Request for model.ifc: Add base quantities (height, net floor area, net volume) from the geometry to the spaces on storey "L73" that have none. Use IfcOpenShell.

First a look at what the model holds.

```python
import ifcopenshell
import ifcopenshell.util.element
import ifcopenshell.util.unit

model = ifcopenshell.open("model.ifc")
print(model.schema)
for unit_type in ("LENGTHUNIT", "AREAUNIT", "VOLUMEUNIT"):
    print(unit_type, ifcopenshell.util.unit.calculate_unit_scale(model, unit_type))
storey = next(s for s in model.by_type("IfcBuildingStorey") if s.Name == "L73")
spaces = [e for e in ifcopenshell.util.element.get_decomposition(storey) if e.is_a("IfcSpace")]
for e in sorted(spaces, key=lambda e: e.id()):
    print(e.id(), e.is_a(), e.Name, list(ifcopenshell.util.element.get_psets(e, qtos_only=True)), sep=" | ")
```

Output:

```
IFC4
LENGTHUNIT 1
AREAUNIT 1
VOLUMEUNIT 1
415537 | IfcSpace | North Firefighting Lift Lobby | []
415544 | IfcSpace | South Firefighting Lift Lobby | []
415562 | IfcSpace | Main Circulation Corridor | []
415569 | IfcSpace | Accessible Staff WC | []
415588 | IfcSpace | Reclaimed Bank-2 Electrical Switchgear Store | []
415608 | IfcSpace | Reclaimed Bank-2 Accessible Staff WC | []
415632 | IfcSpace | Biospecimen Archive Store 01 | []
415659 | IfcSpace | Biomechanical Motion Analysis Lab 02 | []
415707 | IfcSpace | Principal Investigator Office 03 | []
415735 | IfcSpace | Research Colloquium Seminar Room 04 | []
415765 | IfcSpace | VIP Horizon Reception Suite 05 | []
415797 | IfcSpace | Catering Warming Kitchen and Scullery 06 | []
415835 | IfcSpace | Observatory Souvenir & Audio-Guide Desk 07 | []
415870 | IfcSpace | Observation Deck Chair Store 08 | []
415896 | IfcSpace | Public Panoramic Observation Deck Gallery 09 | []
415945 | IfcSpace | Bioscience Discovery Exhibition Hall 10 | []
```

```python
import ifcopenshell
import ifcopenshell.api.pset
import ifcopenshell.geom
import ifcopenshell.util.element
import ifcopenshell.util.shape
import ifcopenshell.util.unit

model = ifcopenshell.open("model.ifc")
unit_scale = ifcopenshell.util.unit.calculate_unit_scale(model)
area_scale = ifcopenshell.util.unit.calculate_unit_scale(model, "AREAUNIT")
volume_scale = ifcopenshell.util.unit.calculate_unit_scale(model, "VOLUMEUNIT")
settings = ifcopenshell.geom.settings()

storey = next(s for s in model.by_type("IfcBuildingStorey") if s.Name == "L73")
spaces = [e for e in ifcopenshell.util.element.get_decomposition(storey) if e.is_a("IfcSpace")]

for e in sorted(spaces, key=lambda e: e.id()):
    if ifcopenshell.util.element.get_psets(e, qtos_only=True, should_inherit=False):
        continue
    # Geometry comes back in metres, in the element's own axes.
    shape = ifcopenshell.geom.create_shape(settings, e)
    values = {
        "Height": ifcopenshell.util.shape.get_z(shape.geometry) / unit_scale,
        "NetFloorArea": ifcopenshell.util.shape.get_footprint_area(shape.geometry) / area_scale,
        "NetVolume": ifcopenshell.util.shape.get_volume(shape.geometry) / volume_scale,
    }
    qto = ifcopenshell.api.pset.add_qto(model, product=e, name="Qto_SpaceBaseQuantities")
    ifcopenshell.api.pset.edit_qto(model, qto=qto, properties=values)
    print(e.id(), {k: round(v, 3) for k, v in values.items()})

model.write("model_edited.ifc")
```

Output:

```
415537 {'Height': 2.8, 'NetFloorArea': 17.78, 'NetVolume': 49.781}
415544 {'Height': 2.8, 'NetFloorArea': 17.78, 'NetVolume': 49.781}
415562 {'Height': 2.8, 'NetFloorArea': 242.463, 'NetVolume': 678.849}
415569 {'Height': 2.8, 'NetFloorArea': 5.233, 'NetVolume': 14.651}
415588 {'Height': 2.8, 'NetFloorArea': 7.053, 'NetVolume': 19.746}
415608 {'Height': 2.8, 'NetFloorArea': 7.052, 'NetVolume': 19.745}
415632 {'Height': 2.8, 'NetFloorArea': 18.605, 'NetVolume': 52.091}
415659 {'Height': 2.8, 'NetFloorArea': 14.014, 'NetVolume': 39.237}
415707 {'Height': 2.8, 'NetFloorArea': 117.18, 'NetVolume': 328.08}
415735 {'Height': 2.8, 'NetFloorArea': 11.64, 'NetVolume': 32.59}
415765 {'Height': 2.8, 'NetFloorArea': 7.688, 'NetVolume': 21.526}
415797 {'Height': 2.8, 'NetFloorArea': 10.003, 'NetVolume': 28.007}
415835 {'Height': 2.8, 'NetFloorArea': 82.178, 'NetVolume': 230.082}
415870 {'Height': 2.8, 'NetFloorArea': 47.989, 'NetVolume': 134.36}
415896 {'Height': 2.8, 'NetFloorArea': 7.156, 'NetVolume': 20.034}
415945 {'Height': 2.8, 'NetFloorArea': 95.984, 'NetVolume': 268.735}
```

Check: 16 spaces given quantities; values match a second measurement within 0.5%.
